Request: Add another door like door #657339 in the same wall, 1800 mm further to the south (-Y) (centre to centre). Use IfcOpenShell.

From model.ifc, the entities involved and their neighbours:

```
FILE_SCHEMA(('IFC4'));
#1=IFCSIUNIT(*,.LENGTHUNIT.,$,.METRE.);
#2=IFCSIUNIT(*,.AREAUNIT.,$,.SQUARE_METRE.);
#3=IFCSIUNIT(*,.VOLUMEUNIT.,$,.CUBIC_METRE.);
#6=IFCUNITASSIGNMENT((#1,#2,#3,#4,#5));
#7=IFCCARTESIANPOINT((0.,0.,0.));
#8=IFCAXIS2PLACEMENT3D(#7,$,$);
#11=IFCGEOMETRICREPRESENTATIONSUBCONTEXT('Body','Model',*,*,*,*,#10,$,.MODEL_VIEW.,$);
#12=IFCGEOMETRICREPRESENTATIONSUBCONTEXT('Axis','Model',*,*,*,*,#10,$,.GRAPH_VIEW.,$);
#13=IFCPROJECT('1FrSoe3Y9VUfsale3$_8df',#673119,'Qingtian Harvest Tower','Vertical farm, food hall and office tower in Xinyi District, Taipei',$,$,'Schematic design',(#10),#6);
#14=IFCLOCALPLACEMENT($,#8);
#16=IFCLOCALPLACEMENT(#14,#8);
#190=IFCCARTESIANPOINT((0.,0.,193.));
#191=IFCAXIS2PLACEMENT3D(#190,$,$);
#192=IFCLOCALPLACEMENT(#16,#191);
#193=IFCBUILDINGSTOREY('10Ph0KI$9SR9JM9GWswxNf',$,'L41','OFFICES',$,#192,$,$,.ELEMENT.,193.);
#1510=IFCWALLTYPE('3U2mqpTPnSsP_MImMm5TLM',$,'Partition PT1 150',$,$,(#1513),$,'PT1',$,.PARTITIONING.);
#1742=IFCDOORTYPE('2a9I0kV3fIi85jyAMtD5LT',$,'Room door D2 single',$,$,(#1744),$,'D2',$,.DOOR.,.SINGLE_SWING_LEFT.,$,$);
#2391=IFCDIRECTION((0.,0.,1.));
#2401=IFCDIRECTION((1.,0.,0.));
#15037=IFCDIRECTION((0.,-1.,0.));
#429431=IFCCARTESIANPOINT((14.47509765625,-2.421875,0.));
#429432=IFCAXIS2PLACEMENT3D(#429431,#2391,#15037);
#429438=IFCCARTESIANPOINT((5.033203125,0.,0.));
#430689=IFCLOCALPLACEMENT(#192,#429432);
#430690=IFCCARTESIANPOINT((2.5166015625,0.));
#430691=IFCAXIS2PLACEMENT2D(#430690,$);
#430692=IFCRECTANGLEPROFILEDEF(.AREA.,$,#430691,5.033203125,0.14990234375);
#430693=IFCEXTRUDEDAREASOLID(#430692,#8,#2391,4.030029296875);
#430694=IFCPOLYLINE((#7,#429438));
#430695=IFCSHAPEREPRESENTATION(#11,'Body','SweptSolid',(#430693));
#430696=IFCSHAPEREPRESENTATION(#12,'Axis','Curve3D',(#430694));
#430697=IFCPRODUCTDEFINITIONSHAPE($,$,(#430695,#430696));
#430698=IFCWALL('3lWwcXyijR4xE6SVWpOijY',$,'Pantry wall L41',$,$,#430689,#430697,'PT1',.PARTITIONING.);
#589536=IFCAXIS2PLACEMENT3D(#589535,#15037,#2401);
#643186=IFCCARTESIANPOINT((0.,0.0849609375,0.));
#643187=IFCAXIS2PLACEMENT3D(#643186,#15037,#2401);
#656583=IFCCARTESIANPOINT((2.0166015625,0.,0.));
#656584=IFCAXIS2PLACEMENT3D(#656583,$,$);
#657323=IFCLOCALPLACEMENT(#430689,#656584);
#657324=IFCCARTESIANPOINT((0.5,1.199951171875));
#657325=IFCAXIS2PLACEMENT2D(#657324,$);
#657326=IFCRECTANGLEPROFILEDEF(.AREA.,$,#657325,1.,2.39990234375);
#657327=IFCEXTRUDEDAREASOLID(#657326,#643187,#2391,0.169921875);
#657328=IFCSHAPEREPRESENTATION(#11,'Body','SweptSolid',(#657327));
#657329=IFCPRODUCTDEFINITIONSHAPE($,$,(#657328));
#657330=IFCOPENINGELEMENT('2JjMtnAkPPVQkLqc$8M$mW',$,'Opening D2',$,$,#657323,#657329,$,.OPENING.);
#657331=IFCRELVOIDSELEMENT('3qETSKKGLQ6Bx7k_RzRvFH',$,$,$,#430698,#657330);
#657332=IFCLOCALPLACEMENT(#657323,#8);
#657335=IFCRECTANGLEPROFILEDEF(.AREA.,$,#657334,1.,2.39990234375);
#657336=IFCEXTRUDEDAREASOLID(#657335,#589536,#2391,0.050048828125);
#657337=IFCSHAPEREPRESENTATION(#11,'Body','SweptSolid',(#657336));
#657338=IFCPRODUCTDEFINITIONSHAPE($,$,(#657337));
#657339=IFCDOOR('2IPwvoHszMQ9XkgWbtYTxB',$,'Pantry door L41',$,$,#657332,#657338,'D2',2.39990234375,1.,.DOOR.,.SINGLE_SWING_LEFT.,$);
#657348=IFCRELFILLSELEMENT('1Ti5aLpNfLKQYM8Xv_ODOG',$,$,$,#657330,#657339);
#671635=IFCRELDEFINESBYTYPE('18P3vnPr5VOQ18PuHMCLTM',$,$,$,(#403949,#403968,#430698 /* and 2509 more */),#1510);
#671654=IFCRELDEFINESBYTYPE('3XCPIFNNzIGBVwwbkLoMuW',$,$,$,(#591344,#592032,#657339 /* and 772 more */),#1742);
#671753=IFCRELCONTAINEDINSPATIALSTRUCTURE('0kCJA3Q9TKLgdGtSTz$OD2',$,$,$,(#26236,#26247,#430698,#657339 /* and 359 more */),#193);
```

```python
import ifcopenshell
import ifcopenshell.api.feature
import ifcopenshell.api.geometry
import ifcopenshell.api.root
import ifcopenshell.geom
import ifcopenshell.util.element
import ifcopenshell.util.placement
import ifcopenshell.util.shape
import ifcopenshell.util.unit

model = ifcopenshell.open("model.ifc")
unit_scale = ifcopenshell.util.unit.calculate_unit_scale(model)
settings = ifcopenshell.geom.settings()


def volume(element):
    """Net volume in cubic metres, openings subtracted."""
    shape = ifcopenshell.geom.create_shape(settings, element)
    return ifcopenshell.util.shape.get_volume(shape.geometry)


door = model.by_guid("2IPwvoHszMQ9XkgWbtYTxB")
opening = door.FillsVoids[0].RelatingOpeningElement
wall = opening.VoidsElements[0].RelatingBuildingElement
before = volume(wall)
shift = ifcopenshell.util.placement.get_local_placement(wall.ObjectPlacement)[:3, 0] * 1.8 / unit_scale

# copy_class copies the void relationship, type, container and properties, but no geometry.
new_opening = ifcopenshell.api.root.copy_class(model, product=opening)
new_opening.Representation = ifcopenshell.util.element.copy_deep(
    model, opening.Representation, exclude=["IfcGeometricRepresentationContext", "IfcRepresentationMap"]
)
new_door = ifcopenshell.api.root.copy_class(model, product=door)
new_door.Representation = ifcopenshell.util.element.copy_deep(
    model, door.Representation, exclude=["IfcGeometricRepresentationContext", "IfcRepresentationMap"]
)
new_door.Tag = None
ifcopenshell.api.feature.add_filling(model, opening=new_opening, element=new_door)

for old, new in ((opening, new_opening), (door, new_door)):
    matrix = ifcopenshell.util.placement.get_local_placement(old.ObjectPlacement)
    matrix[:3, 3] += shift
    ifcopenshell.api.geometry.edit_object_placement(model, product=new, matrix=matrix, is_si=False)

after = volume(wall)

print(f"wall volume {before:.3f} -> {after:.3f} m3")

model.write("model_edited.ifc")
```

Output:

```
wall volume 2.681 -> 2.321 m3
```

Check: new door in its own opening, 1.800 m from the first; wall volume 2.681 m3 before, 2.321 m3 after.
